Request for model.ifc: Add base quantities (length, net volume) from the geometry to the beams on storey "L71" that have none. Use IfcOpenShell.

First a look at what the model holds.

```python
import ifcopenshell
import ifcopenshell.util.element
import ifcopenshell.util.unit

model = ifcopenshell.open("model.ifc")
print(model.schema)
for unit_type in ("LENGTHUNIT", "AREAUNIT", "VOLUMEUNIT"):
    print(unit_type, ifcopenshell.util.unit.calculate_unit_scale(model, unit_type))
storey = next(s for s in model.by_type("IfcBuildingStorey") if s.Name == "L71")
beams = [e for e in ifcopenshell.util.element.get_decomposition(storey) if e.is_a("IfcBeam")]
for e in sorted(beams, key=lambda e: e.id()):
    print(e.id(), e.is_a(), e.Name, list(ifcopenshell.util.element.get_psets(e, qtos_only=True)), sep=" | ")
```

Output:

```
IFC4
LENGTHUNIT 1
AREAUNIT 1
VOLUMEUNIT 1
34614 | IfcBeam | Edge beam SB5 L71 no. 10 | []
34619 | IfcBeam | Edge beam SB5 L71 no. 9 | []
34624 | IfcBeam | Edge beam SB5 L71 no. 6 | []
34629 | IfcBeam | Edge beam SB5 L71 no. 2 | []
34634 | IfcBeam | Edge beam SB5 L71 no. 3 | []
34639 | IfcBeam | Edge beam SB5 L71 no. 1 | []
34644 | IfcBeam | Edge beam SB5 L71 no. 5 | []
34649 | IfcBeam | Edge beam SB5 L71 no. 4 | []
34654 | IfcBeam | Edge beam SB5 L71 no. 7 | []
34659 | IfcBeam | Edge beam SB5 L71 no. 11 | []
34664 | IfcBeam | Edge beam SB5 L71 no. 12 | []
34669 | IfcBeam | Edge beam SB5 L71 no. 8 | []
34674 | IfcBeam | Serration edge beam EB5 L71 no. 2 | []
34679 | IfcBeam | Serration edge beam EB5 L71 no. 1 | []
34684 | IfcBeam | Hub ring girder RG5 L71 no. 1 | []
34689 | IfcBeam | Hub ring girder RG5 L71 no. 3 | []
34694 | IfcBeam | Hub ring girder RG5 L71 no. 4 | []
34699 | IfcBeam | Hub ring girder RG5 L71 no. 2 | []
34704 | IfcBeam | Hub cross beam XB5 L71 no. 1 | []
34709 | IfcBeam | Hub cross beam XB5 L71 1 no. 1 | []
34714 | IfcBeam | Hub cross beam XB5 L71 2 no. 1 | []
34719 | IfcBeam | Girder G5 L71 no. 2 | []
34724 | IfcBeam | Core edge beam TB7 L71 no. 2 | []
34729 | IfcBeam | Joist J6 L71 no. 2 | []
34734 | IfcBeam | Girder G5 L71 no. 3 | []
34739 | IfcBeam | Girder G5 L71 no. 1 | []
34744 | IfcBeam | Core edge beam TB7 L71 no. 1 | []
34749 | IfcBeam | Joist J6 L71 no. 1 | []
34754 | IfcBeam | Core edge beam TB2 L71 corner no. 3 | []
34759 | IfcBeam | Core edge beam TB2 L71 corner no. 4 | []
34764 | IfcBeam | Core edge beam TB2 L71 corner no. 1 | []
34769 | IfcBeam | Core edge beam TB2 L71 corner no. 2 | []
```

```python
import ifcopenshell
import ifcopenshell.api.pset
import ifcopenshell.geom
import ifcopenshell.util.element
import ifcopenshell.util.shape
import ifcopenshell.util.unit

model = ifcopenshell.open("model.ifc")
unit_scale = ifcopenshell.util.unit.calculate_unit_scale(model)
volume_scale = ifcopenshell.util.unit.calculate_unit_scale(model, "VOLUMEUNIT")
settings = ifcopenshell.geom.settings()

storey = next(s for s in model.by_type("IfcBuildingStorey") if s.Name == "L71")
beams = [e for e in ifcopenshell.util.element.get_decomposition(storey) if e.is_a("IfcBeam")]

for e in sorted(beams, key=lambda e: e.id()):
    if ifcopenshell.util.element.get_psets(e, qtos_only=True, should_inherit=False):
        continue
    # Geometry comes back in metres, in the element's own axes.
    shape = ifcopenshell.geom.create_shape(settings, e)
    values = {
        "Length": ifcopenshell.util.shape.get_max_xyz(shape.geometry) / unit_scale,
        "NetVolume": ifcopenshell.util.shape.get_volume(shape.geometry) / volume_scale,
    }
    qto = ifcopenshell.api.pset.add_qto(model, product=e, name="Qto_BeamBaseQuantities")
    ifcopenshell.api.pset.edit_qto(model, qto=qto, properties=values)
    print(e.id(), {k: round(v, 3) for k, v in values.items()})

model.write("model-out.ifc")
```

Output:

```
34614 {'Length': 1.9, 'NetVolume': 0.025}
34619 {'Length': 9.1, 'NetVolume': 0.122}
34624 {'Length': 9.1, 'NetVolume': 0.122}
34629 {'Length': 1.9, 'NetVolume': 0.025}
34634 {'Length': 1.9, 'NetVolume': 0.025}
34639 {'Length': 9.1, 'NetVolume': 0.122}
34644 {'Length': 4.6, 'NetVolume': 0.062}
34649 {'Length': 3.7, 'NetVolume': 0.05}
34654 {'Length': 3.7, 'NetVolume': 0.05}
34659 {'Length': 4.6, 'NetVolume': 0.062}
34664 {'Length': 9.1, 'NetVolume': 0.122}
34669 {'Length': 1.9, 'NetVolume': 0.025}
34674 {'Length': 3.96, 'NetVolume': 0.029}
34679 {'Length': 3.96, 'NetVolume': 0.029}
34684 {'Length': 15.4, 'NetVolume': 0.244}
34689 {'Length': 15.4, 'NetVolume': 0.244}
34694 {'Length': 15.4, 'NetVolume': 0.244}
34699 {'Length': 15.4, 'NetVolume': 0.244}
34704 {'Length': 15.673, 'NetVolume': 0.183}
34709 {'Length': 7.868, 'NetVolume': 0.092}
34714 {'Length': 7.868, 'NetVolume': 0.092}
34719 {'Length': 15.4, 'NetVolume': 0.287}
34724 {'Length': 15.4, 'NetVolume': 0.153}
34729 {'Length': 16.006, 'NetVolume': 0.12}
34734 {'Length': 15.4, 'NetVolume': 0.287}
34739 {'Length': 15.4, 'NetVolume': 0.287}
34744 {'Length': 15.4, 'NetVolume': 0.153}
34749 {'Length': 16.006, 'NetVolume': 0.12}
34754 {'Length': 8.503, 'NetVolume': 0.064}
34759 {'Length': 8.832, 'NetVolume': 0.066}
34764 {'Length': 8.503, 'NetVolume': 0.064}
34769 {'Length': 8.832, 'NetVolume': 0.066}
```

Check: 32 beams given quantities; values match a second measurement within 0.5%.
